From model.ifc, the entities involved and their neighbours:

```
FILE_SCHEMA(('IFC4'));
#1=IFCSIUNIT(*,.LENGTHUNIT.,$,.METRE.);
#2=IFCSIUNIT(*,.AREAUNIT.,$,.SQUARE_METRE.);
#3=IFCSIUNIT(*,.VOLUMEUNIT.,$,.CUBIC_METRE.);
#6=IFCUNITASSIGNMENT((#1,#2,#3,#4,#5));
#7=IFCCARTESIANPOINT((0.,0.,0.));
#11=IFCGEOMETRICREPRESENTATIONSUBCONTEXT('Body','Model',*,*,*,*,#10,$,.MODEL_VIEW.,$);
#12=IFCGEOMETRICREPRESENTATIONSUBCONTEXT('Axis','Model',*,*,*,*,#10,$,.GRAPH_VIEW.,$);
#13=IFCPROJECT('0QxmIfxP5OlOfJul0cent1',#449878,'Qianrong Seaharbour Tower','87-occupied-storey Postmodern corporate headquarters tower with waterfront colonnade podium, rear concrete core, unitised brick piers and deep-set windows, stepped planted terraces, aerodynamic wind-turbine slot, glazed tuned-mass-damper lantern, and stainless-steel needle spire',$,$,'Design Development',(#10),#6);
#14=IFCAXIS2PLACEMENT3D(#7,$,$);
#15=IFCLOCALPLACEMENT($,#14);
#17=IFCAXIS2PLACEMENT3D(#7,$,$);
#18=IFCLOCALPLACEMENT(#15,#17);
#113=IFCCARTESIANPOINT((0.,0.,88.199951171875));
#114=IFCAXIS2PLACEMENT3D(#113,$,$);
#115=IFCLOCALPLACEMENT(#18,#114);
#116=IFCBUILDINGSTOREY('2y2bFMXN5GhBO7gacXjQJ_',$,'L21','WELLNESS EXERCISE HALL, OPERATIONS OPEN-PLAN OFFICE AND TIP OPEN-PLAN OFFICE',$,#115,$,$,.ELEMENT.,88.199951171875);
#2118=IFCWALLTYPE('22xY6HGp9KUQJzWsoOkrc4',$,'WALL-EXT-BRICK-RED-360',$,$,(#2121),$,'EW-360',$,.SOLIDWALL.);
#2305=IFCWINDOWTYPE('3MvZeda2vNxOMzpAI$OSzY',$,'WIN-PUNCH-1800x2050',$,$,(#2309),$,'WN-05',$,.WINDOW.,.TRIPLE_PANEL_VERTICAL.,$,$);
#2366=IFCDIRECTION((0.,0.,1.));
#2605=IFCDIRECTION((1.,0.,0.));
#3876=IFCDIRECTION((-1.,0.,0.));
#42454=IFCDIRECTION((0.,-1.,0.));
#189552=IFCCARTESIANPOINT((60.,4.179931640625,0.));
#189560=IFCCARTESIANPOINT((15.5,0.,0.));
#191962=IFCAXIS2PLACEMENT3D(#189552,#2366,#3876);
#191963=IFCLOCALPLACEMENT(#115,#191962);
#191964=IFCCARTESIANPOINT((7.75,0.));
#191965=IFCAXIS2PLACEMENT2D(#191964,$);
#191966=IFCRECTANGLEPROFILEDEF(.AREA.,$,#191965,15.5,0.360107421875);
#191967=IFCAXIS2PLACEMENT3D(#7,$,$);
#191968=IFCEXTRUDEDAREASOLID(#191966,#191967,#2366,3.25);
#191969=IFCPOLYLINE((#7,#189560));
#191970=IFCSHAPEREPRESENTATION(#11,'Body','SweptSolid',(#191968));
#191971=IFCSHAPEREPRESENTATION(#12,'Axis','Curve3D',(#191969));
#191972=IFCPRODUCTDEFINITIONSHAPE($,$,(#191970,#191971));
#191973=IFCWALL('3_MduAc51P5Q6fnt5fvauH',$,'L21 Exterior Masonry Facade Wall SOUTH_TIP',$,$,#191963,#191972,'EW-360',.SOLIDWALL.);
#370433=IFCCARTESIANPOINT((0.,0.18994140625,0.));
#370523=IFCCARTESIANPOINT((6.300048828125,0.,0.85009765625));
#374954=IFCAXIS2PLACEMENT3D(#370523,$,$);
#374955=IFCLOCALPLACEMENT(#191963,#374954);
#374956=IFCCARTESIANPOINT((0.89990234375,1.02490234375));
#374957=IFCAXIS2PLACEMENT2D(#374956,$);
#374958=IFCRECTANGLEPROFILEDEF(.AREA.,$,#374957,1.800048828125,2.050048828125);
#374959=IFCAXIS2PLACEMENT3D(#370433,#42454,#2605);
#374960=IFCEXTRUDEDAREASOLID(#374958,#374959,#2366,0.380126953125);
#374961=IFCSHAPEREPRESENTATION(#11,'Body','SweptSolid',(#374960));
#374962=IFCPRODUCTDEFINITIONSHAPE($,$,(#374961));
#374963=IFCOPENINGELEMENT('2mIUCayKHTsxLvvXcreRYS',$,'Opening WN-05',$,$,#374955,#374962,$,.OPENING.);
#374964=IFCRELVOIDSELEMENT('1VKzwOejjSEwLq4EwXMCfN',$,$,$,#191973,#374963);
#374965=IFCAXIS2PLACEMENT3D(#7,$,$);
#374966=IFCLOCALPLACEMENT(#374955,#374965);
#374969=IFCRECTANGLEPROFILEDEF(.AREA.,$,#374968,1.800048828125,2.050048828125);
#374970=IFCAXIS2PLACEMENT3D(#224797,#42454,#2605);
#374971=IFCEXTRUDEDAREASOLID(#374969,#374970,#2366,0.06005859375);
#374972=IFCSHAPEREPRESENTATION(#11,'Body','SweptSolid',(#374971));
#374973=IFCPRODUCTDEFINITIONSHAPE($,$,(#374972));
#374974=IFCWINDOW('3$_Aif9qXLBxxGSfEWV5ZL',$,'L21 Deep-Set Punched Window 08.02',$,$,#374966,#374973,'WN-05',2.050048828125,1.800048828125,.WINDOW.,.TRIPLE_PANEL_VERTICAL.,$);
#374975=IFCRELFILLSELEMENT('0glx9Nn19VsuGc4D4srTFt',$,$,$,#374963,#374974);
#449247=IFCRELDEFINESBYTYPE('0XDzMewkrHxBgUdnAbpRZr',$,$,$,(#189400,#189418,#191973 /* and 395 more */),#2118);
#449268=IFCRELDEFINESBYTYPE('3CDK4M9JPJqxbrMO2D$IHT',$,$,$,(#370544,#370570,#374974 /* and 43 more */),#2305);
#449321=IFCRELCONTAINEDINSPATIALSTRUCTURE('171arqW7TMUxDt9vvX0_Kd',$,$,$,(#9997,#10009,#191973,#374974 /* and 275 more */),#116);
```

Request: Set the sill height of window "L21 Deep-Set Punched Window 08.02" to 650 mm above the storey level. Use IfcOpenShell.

```python
import numpy as np
import ifcopenshell
import ifcopenshell.api.geometry
import ifcopenshell.geom
import ifcopenshell.util.element
import ifcopenshell.util.placement
import ifcopenshell.util.shape
import ifcopenshell.util.unit

model = ifcopenshell.open("model.ifc")
unit_scale = ifcopenshell.util.unit.calculate_unit_scale(model)

window = model.by_id(374974)
opening = window.FillsVoids[0].RelatingOpeningElement
storey = ifcopenshell.util.element.get_container(window, ifc_class="IfcBuildingStorey")
level = ifcopenshell.util.placement.get_local_placement(storey.ObjectPlacement)[2, 3]

# The opening's origin need not be at the sill, so measure its lowest point.
shape = ifcopenshell.geom.create_shape(ifcopenshell.geom.settings(), opening)
bottom = ifcopenshell.util.shape.get_shape_bottom_elevation(shape, shape.geometry) / unit_scale
dz = level + 0.65 / unit_scale - bottom

shift = np.array([0.0, 0.0, dz])
# The window is placed relative to its opening, so it follows when the opening moves.
matrix = ifcopenshell.util.placement.get_local_placement(opening.ObjectPlacement)
matrix[:3, 3] += shift
ifcopenshell.api.geometry.edit_object_placement(
    model, product=opening, matrix=matrix, is_si=False, should_transform_children=True
)

print(f"moved by {dz * unit_scale:+.3f} m")

model.write("model_v2.ifc")
```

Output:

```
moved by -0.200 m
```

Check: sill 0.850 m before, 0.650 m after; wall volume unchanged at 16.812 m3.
